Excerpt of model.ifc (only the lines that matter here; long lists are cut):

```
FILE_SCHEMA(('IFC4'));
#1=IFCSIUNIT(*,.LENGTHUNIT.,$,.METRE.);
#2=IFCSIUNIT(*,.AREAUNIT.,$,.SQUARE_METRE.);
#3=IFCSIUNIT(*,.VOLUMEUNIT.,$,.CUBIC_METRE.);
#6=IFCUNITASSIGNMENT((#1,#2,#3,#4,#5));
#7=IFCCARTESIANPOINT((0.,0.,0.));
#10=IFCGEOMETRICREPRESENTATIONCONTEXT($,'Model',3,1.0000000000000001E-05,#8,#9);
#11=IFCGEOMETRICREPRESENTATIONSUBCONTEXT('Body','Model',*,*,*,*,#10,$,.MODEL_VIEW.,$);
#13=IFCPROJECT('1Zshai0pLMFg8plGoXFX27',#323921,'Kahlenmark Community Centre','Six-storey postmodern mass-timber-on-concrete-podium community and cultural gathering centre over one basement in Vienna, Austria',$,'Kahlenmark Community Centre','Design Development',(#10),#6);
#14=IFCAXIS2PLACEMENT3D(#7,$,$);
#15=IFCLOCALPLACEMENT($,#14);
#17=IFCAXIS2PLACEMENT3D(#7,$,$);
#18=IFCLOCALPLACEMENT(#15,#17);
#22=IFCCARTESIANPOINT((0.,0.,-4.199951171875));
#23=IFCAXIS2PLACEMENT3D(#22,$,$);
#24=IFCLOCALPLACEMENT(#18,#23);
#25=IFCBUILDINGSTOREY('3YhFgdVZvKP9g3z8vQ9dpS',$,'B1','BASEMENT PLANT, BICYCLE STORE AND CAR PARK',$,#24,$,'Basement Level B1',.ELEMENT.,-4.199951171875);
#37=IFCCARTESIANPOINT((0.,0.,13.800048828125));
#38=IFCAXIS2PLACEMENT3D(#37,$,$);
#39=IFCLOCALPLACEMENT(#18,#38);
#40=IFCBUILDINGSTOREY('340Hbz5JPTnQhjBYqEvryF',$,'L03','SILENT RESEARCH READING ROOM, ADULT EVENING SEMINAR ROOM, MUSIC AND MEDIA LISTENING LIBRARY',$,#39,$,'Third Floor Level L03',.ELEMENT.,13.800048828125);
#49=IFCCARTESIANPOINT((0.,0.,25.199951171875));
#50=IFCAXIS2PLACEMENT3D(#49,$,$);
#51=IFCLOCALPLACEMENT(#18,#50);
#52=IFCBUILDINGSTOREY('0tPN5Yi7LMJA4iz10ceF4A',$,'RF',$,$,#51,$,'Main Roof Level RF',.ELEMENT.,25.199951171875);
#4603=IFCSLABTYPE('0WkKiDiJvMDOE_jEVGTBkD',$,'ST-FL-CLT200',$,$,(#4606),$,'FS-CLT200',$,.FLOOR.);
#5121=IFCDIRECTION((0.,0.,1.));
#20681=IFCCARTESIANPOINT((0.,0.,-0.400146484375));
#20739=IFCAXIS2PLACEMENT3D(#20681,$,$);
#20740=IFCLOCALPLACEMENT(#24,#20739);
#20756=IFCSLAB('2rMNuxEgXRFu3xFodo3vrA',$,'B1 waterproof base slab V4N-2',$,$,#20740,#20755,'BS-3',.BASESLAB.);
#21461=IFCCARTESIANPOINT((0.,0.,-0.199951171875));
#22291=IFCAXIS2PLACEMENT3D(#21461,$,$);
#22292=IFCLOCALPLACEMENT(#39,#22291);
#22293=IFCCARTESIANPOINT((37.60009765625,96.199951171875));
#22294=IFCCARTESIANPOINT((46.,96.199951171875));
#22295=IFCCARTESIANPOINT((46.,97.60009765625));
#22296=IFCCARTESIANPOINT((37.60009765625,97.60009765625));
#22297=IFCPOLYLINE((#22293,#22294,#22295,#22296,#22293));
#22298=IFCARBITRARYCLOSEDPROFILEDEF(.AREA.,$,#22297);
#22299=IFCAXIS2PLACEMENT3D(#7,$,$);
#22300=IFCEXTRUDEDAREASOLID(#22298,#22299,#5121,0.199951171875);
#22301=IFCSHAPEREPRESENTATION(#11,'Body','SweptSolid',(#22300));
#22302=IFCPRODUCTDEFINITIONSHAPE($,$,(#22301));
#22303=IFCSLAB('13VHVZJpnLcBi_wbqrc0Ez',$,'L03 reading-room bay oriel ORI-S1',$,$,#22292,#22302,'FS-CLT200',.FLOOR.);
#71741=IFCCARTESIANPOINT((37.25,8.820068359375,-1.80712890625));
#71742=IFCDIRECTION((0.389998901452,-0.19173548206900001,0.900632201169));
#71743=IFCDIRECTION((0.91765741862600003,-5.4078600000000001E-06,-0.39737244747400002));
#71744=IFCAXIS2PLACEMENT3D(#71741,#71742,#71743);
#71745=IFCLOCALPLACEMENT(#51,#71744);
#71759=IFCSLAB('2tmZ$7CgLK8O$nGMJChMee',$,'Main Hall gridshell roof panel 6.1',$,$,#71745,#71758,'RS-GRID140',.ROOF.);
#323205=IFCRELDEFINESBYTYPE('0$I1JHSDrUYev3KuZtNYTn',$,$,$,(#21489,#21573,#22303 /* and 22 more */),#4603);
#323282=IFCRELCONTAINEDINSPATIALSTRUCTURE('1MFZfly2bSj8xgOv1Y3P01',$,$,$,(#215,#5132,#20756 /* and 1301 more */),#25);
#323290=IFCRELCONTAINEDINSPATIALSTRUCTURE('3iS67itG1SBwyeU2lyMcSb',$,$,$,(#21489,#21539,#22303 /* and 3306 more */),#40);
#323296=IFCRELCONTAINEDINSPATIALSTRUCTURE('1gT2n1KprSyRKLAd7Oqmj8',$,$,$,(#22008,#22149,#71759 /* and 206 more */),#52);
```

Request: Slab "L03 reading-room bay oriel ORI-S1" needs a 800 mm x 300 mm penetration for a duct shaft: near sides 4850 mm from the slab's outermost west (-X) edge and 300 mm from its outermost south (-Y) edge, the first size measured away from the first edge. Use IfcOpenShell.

```python
import numpy as np
import ifcopenshell
import ifcopenshell.api.feature
import ifcopenshell.api.geometry
import ifcopenshell.api.root
import ifcopenshell.geom
import ifcopenshell.util.placement
import ifcopenshell.util.representation
import ifcopenshell.util.shape
import ifcopenshell.util.unit

model = ifcopenshell.open("model.ifc")
unit_scale = ifcopenshell.util.unit.calculate_unit_scale(model)
settings = ifcopenshell.geom.settings()


def volume(element):
    """Net volume in cubic metres, openings subtracted."""
    shape = ifcopenshell.geom.create_shape(settings, element)
    return ifcopenshell.util.shape.get_volume(shape.geometry)


slab = model.by_guid("13VHVZJpnLcBi_wbqrc0Ez")
before = volume(slab)

# Extent in the slab's own axes, in metres. The edges named are its -X and -Y sides.
slab_shape = ifcopenshell.geom.create_shape(settings, slab)
vertices = ifcopenshell.util.shape.get_vertices(slab_shape.geometry)
x_min, y_min, bottom = vertices.min(axis=0)
top = vertices[:, 2].max()

opening = ifcopenshell.api.root.create_entity(model, ifc_class="IfcOpeningElement", name="Duct shaft opening", predefined_type="OPENING")
context = ifcopenshell.util.representation.get_context(model, "Model", "Body", "MODEL_VIEW")
width, depth = 0.8, 0.3
outline = [(0.0, 0.0), (width, 0.0), (width, depth), (0.0, depth), (0.0, 0.0)]
# Overshoot both faces by 50 mm so the cut is clean.
shape = ifcopenshell.api.geometry.add_slab_representation(
    model, context=context, depth=top - bottom + 0.1, polyline=outline
)
ifcopenshell.api.geometry.assign_representation(model, product=opening, representation=shape)

matrix = ifcopenshell.util.placement.get_local_placement(slab.ObjectPlacement)
matrix[:, 3] = matrix @ np.append(np.array([x_min + 4.85, y_min + 0.3, bottom - 0.05]) / unit_scale, 1.0)
ifcopenshell.api.geometry.edit_object_placement(model, product=opening, matrix=matrix, is_si=False)
ifcopenshell.api.feature.add_feature(model, feature=opening, element=slab)

after = volume(slab)

print(f"slab volume {before:.3f} -> {after:.3f} m3")

model.write("model_rev.ifc")
```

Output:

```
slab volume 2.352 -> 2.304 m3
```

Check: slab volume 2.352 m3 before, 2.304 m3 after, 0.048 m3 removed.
